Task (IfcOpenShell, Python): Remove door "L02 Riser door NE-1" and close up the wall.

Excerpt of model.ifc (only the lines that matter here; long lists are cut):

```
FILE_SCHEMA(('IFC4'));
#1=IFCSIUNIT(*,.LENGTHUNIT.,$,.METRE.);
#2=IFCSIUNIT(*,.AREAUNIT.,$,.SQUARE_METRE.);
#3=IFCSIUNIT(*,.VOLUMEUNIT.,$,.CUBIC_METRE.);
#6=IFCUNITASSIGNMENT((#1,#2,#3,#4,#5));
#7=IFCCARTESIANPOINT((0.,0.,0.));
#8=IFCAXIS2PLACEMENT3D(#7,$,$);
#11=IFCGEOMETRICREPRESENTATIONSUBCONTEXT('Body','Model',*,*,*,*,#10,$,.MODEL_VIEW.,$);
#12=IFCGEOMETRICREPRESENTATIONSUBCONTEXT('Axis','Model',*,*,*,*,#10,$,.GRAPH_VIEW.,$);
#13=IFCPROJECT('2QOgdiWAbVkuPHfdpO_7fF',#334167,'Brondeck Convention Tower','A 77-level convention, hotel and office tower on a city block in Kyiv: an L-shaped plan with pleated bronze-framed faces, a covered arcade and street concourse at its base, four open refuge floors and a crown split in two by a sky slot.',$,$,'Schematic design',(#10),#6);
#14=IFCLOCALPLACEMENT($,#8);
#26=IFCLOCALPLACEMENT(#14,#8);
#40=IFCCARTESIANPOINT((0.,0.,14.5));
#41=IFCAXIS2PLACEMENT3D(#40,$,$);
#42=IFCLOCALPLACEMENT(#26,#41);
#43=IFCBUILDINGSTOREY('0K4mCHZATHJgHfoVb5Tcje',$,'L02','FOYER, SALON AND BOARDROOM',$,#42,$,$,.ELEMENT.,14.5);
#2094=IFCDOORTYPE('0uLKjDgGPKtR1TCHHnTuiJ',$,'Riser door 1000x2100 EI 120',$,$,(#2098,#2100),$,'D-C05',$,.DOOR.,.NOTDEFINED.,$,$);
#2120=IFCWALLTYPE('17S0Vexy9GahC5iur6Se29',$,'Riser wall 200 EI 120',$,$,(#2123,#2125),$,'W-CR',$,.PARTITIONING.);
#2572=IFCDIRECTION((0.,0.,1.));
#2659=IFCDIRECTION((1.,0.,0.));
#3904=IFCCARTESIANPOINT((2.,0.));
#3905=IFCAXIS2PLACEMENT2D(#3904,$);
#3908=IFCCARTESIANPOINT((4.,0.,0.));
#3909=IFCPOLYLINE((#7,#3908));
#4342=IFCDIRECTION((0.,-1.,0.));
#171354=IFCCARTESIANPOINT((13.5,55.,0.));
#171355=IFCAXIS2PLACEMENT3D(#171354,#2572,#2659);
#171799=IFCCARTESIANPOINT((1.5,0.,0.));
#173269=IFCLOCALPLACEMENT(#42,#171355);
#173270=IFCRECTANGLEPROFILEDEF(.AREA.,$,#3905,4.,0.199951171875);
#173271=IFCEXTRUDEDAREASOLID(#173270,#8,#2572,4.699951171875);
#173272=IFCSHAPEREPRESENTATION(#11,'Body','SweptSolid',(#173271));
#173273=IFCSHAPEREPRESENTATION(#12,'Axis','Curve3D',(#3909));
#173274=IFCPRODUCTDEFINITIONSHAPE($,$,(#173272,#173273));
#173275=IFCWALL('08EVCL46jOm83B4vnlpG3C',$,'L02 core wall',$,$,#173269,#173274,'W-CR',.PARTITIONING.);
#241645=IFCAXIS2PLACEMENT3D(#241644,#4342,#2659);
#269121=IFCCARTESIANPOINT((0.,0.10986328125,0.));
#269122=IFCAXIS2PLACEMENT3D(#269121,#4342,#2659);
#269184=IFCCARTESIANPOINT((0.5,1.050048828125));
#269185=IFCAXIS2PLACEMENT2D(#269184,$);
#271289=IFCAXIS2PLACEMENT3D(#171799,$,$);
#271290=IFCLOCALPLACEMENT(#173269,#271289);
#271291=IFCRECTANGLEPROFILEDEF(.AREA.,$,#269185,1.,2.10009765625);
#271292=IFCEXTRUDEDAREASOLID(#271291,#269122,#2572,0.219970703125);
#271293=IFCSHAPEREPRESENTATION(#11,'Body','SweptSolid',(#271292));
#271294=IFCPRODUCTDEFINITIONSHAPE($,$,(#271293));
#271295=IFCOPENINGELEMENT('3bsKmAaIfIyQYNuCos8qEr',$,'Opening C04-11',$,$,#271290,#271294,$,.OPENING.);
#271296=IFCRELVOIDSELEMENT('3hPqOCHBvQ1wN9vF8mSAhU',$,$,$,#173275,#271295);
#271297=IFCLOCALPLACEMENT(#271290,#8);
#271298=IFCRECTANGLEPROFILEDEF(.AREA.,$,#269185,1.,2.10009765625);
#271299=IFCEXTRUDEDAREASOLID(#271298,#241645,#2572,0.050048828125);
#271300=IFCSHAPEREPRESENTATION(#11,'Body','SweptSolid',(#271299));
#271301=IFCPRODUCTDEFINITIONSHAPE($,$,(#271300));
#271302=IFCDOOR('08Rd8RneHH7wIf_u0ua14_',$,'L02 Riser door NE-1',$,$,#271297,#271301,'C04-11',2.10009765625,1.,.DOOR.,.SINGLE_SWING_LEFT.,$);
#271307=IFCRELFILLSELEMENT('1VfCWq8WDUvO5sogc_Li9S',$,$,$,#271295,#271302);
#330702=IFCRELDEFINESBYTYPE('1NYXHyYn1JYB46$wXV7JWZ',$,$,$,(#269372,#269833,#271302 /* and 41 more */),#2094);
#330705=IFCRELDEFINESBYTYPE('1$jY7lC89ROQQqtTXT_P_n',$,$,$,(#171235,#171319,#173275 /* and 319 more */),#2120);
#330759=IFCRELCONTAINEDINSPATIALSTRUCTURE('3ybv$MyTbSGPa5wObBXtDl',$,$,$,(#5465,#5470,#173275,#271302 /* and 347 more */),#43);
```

```python
import ifcopenshell
import ifcopenshell.api.feature
import ifcopenshell.api.root
import ifcopenshell.geom
import ifcopenshell.util.shape

model = ifcopenshell.open("model.ifc")
settings = ifcopenshell.geom.settings()


def volume(element):
    """Net volume in cubic metres, openings subtracted."""
    shape = ifcopenshell.geom.create_shape(settings, element)
    return ifcopenshell.util.shape.get_volume(shape.geometry)


door = model.by_guid("08Rd8RneHH7wIf_u0ua14_")
opening = door.FillsVoids[0].RelatingOpeningElement
wall = opening.VoidsElements[0].RelatingBuildingElement
before = volume(wall)

ifcopenshell.api.root.remove_product(model, product=door)
ifcopenshell.api.feature.remove_feature(model, feature=opening)

after = volume(wall)

print(f"wall volume {before:.3f} -> {after:.3f} m3")

model.write("model_updated.ifc")
```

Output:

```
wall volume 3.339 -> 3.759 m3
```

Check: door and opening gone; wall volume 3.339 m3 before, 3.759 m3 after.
